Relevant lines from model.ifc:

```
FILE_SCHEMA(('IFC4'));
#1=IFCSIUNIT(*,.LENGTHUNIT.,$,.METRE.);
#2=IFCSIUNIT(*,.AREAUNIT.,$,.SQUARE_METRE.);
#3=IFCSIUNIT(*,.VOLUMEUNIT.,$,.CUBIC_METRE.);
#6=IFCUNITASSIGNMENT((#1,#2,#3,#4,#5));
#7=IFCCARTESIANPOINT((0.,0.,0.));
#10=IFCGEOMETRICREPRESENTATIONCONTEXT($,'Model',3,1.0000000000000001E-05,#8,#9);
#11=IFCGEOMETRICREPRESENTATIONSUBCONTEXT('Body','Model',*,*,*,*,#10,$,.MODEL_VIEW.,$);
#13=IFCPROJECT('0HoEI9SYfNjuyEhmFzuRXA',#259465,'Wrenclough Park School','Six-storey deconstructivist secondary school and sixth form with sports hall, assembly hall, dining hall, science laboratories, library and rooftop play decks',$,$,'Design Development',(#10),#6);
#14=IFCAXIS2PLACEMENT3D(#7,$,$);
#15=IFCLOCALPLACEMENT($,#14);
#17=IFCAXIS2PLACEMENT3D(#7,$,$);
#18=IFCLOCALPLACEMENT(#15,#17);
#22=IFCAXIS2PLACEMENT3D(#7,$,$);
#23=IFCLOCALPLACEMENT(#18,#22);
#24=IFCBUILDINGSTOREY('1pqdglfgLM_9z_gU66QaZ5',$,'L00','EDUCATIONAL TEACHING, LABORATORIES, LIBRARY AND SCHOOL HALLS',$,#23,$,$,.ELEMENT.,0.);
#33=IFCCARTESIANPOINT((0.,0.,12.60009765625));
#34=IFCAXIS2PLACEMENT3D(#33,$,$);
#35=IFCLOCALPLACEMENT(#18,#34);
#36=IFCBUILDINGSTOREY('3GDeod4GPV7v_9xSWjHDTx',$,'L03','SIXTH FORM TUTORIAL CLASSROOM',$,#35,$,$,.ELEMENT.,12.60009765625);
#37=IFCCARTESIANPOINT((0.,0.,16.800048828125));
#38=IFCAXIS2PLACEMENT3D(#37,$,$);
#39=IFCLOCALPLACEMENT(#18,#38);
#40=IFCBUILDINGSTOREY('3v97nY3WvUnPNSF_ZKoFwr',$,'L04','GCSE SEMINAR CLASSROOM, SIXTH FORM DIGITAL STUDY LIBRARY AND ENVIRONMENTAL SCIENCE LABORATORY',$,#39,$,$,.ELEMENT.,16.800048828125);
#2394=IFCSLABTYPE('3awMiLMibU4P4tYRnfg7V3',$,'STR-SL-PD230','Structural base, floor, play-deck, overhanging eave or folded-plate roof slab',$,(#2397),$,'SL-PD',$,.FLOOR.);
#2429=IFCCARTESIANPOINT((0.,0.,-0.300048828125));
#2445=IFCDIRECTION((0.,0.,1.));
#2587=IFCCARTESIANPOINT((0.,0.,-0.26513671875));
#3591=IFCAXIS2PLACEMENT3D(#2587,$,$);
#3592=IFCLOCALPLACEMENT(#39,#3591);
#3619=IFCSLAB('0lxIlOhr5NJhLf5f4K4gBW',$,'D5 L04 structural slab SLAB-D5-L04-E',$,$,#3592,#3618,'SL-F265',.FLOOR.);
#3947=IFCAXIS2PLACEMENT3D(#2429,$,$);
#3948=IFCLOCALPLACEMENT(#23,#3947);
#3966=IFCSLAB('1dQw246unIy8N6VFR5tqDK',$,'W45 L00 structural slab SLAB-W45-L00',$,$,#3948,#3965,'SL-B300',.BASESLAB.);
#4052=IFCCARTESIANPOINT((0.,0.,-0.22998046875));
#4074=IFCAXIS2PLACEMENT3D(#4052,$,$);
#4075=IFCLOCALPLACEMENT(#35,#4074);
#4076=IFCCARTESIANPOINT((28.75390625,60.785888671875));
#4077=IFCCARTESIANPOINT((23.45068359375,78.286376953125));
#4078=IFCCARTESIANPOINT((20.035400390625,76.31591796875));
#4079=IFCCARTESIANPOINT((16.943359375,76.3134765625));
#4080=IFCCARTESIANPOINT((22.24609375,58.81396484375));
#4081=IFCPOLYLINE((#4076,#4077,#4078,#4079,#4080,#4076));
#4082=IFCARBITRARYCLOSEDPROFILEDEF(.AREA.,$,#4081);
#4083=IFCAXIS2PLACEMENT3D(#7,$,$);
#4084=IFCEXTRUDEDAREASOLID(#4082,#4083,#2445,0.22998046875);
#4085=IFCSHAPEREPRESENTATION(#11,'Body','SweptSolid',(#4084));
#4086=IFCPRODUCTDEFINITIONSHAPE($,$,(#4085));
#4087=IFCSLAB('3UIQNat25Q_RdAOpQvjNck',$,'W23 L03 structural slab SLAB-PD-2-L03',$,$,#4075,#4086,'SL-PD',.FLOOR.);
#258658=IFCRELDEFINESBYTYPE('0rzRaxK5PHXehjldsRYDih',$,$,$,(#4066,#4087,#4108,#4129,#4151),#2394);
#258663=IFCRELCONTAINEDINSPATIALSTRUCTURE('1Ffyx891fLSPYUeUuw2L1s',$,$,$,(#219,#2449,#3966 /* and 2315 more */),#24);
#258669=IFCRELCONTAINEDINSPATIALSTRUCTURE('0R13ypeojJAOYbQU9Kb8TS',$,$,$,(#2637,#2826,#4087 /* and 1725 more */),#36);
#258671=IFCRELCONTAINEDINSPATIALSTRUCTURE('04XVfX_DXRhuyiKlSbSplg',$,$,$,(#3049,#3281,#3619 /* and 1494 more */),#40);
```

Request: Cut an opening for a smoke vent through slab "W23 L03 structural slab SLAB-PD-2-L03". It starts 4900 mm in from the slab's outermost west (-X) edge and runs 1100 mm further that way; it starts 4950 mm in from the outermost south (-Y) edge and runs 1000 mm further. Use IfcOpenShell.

```python
import numpy as np
import ifcopenshell
import ifcopenshell.api.feature
import ifcopenshell.api.geometry
import ifcopenshell.api.root
import ifcopenshell.geom
import ifcopenshell.util.placement
import ifcopenshell.util.representation
import ifcopenshell.util.shape
import ifcopenshell.util.unit

model = ifcopenshell.open("model.ifc")
unit_scale = ifcopenshell.util.unit.calculate_unit_scale(model)
settings = ifcopenshell.geom.settings()


def volume(element):
    """Net volume in cubic metres, openings subtracted."""
    shape = ifcopenshell.geom.create_shape(settings, element)
    return ifcopenshell.util.shape.get_volume(shape.geometry)


slab = model.by_id(4087)
before = volume(slab)

# Extent in the slab's own axes, in metres. The edges named are its -X and -Y sides.
slab_shape = ifcopenshell.geom.create_shape(settings, slab)
vertices = ifcopenshell.util.shape.get_vertices(slab_shape.geometry)
x_min, y_min, bottom = vertices.min(axis=0)
top = vertices[:, 2].max()

opening = ifcopenshell.api.root.create_entity(model, ifc_class="IfcOpeningElement", name="Smoke vent opening", predefined_type="OPENING")
context = ifcopenshell.util.representation.get_context(model, "Model", "Body", "MODEL_VIEW")
width, depth = 1.1, 1
outline = [(0.0, 0.0), (width, 0.0), (width, depth), (0.0, depth), (0.0, 0.0)]
# Overshoot both faces by 50 mm so the cut is clean.
shape = ifcopenshell.api.geometry.add_slab_representation(
    model, context=context, depth=top - bottom + 0.1, polyline=outline
)
ifcopenshell.api.geometry.assign_representation(model, product=opening, representation=shape)

matrix = ifcopenshell.util.placement.get_local_placement(slab.ObjectPlacement)
matrix[:, 3] = matrix @ np.append(np.array([x_min + 4.9, y_min + 4.95, bottom - 0.05]) / unit_scale, 1.0)
ifcopenshell.api.geometry.edit_object_placement(model, product=opening, matrix=matrix, is_si=False)
ifcopenshell.api.feature.add_feature(model, feature=opening, element=slab)

after = volume(slab)

print(f"slab volume {before:.3f} -> {after:.3f} m3")

model.write("model_edited.ifc")
```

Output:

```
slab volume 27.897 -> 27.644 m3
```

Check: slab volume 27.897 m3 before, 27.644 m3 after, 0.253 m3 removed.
